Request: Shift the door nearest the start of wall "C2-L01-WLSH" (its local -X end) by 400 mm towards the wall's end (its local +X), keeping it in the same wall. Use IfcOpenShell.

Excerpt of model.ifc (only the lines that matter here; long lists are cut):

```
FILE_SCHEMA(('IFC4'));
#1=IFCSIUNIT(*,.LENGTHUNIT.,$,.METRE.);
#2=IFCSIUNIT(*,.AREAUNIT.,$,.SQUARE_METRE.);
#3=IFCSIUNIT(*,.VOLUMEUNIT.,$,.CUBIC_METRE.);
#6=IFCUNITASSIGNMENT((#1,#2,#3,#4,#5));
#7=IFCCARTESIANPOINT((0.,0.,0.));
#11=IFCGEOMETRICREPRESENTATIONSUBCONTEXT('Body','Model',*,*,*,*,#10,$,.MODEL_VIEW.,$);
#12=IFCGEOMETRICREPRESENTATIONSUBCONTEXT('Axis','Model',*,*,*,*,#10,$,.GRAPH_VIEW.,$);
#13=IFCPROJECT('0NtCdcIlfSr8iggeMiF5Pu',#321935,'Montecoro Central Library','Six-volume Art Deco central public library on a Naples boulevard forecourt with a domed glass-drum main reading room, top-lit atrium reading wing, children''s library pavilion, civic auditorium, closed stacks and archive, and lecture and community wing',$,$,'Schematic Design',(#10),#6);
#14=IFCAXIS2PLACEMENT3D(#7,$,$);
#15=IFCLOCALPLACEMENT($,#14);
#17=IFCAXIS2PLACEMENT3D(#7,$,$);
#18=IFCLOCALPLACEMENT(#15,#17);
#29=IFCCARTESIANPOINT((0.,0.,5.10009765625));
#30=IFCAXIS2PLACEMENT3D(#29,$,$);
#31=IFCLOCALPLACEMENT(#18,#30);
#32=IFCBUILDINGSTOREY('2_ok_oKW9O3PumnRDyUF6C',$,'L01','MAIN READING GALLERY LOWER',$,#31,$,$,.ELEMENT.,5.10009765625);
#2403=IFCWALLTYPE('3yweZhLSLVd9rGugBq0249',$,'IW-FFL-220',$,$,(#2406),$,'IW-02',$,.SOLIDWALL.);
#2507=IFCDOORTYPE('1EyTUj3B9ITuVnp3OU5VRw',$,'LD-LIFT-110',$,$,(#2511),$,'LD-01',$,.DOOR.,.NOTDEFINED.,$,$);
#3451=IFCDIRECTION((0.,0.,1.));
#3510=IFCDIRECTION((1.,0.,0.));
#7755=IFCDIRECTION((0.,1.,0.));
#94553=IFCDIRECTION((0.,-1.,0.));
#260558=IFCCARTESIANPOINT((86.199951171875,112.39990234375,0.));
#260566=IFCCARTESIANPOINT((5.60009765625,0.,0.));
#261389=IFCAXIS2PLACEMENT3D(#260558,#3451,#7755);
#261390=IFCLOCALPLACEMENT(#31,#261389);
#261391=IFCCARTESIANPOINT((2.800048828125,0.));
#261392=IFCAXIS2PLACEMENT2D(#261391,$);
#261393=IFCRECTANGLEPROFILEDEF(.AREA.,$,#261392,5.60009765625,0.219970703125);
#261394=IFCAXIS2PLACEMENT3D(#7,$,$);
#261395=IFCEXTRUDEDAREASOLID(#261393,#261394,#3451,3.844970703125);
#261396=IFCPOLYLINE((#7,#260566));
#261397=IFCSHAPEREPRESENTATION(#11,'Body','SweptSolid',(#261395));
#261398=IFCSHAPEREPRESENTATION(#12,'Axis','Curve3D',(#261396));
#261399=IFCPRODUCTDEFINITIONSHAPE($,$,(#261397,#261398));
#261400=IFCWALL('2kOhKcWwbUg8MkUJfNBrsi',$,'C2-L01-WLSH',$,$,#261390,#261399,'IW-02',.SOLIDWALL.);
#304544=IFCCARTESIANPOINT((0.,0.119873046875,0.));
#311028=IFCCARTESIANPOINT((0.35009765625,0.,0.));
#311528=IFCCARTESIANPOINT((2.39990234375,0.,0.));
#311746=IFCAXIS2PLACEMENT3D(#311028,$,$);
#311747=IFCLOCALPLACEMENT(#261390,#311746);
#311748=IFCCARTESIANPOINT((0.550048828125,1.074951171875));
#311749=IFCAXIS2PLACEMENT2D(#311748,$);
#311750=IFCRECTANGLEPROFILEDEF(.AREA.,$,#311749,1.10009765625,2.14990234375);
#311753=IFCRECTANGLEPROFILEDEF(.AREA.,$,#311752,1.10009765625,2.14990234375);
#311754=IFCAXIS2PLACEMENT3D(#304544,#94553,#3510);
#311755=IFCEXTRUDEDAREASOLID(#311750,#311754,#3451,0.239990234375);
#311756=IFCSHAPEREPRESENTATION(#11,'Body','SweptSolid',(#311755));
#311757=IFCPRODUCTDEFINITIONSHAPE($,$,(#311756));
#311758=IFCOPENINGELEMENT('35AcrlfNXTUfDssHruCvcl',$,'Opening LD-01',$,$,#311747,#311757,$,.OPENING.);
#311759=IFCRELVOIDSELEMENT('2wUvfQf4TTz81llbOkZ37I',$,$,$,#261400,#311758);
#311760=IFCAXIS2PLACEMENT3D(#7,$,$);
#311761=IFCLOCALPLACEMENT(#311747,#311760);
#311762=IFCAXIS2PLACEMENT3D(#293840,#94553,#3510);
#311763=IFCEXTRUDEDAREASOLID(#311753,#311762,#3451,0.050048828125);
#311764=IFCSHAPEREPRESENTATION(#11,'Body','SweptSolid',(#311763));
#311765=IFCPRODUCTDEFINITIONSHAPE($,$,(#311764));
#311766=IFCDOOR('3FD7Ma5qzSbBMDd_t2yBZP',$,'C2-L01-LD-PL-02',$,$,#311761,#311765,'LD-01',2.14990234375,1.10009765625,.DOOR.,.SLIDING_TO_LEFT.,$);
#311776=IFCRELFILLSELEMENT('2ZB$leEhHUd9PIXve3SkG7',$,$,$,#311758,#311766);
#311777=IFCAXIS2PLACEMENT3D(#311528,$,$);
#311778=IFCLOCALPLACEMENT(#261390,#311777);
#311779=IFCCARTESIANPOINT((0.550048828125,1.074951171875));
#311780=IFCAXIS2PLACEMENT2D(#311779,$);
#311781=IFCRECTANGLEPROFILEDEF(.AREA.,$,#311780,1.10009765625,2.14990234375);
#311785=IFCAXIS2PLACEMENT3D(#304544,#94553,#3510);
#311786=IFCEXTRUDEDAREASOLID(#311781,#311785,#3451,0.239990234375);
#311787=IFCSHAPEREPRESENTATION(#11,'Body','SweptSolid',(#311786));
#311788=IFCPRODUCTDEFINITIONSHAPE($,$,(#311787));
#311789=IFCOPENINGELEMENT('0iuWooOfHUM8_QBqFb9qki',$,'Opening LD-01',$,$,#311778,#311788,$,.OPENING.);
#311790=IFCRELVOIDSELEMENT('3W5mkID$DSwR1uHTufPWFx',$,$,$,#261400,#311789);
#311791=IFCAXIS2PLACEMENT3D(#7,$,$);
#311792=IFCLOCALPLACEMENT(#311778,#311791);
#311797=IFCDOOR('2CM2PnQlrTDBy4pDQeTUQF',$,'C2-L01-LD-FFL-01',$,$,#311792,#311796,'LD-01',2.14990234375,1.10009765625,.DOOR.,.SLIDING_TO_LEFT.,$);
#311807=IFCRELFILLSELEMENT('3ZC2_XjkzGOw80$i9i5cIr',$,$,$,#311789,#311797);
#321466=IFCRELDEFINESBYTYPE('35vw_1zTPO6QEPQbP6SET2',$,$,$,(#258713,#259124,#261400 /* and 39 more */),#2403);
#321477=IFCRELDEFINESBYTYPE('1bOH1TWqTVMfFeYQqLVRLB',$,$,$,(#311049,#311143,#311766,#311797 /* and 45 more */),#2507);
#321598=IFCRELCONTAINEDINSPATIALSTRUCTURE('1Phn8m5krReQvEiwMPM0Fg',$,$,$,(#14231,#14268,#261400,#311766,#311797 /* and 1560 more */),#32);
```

```python
import ifcopenshell
import ifcopenshell.api.geometry
import ifcopenshell.util.placement
import ifcopenshell.util.unit

model = ifcopenshell.open("model.ifc")
unit_scale = ifcopenshell.util.unit.calculate_unit_scale(model)

door = model.by_guid("3FD7Ma5qzSbBMDd_t2yBZP")
opening = door.FillsVoids[0].RelatingOpeningElement
wall = opening.VoidsElements[0].RelatingBuildingElement

wall_matrix = ifcopenshell.util.placement.get_local_placement(wall.ObjectPlacement)
shift = wall_matrix[:3, 0] * 0.4 / unit_scale
before = ifcopenshell.util.placement.get_local_placement(door.ObjectPlacement)[:3, 3].copy()

# The door is placed relative to its opening, so it follows when the opening moves.
matrix = ifcopenshell.util.placement.get_local_placement(opening.ObjectPlacement)
matrix[:3, 3] += shift
ifcopenshell.api.geometry.edit_object_placement(
    model, product=opening, matrix=matrix, is_si=False, should_transform_children=True
)

after = ifcopenshell.util.placement.get_local_placement(door.ObjectPlacement)[:3, 3]
print("door moved by", (after - before).round(3) + 0.0)

model.write("model_rev.ifc")
```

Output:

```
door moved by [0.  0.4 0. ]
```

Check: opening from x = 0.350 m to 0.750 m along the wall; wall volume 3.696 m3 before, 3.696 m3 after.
